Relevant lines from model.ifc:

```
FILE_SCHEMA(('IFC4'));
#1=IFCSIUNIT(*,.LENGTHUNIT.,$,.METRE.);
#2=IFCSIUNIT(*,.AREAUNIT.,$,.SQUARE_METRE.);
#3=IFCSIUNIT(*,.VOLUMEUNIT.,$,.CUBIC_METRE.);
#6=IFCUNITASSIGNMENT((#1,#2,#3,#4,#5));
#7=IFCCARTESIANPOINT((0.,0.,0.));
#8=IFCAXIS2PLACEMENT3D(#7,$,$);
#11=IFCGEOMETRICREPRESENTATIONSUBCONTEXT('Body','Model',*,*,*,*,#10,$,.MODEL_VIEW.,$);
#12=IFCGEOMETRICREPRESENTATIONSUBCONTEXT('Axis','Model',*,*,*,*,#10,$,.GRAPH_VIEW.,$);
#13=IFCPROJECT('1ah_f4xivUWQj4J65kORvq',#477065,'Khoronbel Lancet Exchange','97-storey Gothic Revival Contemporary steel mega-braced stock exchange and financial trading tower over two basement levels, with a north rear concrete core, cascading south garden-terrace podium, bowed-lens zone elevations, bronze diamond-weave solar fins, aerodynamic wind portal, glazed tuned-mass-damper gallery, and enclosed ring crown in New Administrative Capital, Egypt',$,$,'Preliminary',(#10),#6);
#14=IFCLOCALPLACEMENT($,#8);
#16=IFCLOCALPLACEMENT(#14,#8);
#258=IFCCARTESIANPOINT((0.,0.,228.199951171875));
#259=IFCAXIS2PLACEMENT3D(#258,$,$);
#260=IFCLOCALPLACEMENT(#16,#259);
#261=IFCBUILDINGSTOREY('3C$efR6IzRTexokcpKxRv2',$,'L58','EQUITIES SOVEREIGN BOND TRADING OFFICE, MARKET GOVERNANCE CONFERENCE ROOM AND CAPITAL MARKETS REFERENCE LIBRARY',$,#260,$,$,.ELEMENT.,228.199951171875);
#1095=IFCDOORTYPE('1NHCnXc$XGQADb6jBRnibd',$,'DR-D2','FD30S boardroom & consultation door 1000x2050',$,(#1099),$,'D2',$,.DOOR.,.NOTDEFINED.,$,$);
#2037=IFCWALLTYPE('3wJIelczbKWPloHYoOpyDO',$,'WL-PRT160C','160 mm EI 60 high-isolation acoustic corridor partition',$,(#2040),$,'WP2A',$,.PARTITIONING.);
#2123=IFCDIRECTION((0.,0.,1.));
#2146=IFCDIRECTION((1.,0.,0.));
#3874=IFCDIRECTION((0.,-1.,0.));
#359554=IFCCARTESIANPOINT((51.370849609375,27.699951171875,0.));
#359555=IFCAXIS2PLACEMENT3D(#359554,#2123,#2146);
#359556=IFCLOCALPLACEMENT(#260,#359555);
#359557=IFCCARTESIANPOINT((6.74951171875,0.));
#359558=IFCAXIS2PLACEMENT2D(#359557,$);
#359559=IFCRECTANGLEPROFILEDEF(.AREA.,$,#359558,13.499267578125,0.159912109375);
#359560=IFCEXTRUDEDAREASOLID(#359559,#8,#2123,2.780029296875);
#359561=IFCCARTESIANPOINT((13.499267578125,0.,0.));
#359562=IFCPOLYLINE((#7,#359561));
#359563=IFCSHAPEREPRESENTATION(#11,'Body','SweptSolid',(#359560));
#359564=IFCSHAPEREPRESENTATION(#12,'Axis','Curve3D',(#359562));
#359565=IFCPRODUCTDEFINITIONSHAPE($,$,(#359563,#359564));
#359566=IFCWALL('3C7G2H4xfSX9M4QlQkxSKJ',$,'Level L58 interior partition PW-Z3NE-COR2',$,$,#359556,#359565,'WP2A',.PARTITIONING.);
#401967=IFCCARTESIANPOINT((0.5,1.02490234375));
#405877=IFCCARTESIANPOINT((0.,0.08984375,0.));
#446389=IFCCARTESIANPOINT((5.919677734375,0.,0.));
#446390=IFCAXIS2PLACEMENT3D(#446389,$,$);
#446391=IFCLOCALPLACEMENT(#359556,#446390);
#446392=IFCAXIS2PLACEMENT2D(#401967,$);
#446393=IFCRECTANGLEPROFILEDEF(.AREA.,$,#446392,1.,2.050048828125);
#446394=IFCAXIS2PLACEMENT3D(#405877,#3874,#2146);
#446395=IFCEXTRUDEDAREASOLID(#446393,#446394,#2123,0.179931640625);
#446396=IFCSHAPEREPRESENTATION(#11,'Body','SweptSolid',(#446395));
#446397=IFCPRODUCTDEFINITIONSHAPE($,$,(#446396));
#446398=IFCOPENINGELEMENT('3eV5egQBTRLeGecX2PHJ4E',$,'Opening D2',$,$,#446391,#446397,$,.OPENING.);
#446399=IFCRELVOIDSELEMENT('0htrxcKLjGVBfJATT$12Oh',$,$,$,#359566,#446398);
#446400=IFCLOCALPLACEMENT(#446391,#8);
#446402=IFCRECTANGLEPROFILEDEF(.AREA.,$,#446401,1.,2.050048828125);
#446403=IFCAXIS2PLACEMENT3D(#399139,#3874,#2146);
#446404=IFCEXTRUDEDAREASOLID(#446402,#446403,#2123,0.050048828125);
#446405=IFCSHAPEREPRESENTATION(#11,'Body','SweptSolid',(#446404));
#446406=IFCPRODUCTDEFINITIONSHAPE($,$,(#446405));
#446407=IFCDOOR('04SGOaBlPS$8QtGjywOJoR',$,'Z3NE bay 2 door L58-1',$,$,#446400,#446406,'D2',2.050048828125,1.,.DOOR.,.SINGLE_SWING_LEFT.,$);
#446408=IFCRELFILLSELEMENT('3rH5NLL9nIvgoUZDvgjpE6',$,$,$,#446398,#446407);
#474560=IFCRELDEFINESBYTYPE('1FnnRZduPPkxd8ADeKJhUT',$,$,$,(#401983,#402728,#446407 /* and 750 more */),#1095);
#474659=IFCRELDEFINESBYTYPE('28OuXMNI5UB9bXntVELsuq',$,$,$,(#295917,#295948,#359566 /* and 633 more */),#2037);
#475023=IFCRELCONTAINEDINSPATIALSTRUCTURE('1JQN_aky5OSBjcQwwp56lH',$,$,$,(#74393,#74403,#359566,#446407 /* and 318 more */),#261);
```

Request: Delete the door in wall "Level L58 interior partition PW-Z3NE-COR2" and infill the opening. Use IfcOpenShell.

```python
import ifcopenshell
import ifcopenshell.api.feature
import ifcopenshell.api.root
import ifcopenshell.geom
import ifcopenshell.util.shape

model = ifcopenshell.open("model.ifc")
settings = ifcopenshell.geom.settings()


def volume(element):
    """Net volume in cubic metres, openings subtracted."""
    shape = ifcopenshell.geom.create_shape(settings, element)
    return ifcopenshell.util.shape.get_volume(shape.geometry)


door = model.by_guid("04SGOaBlPS$8QtGjywOJoR")
opening = door.FillsVoids[0].RelatingOpeningElement
wall = opening.VoidsElements[0].RelatingBuildingElement
before = volume(wall)

ifcopenshell.api.root.remove_product(model, product=door)
ifcopenshell.api.feature.remove_feature(model, feature=opening)

after = volume(wall)

print(f"wall volume {before:.3f} -> {after:.3f} m3")

model.write("model_edited.ifc")
```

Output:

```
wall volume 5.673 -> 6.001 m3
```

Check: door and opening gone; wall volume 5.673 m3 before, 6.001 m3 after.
